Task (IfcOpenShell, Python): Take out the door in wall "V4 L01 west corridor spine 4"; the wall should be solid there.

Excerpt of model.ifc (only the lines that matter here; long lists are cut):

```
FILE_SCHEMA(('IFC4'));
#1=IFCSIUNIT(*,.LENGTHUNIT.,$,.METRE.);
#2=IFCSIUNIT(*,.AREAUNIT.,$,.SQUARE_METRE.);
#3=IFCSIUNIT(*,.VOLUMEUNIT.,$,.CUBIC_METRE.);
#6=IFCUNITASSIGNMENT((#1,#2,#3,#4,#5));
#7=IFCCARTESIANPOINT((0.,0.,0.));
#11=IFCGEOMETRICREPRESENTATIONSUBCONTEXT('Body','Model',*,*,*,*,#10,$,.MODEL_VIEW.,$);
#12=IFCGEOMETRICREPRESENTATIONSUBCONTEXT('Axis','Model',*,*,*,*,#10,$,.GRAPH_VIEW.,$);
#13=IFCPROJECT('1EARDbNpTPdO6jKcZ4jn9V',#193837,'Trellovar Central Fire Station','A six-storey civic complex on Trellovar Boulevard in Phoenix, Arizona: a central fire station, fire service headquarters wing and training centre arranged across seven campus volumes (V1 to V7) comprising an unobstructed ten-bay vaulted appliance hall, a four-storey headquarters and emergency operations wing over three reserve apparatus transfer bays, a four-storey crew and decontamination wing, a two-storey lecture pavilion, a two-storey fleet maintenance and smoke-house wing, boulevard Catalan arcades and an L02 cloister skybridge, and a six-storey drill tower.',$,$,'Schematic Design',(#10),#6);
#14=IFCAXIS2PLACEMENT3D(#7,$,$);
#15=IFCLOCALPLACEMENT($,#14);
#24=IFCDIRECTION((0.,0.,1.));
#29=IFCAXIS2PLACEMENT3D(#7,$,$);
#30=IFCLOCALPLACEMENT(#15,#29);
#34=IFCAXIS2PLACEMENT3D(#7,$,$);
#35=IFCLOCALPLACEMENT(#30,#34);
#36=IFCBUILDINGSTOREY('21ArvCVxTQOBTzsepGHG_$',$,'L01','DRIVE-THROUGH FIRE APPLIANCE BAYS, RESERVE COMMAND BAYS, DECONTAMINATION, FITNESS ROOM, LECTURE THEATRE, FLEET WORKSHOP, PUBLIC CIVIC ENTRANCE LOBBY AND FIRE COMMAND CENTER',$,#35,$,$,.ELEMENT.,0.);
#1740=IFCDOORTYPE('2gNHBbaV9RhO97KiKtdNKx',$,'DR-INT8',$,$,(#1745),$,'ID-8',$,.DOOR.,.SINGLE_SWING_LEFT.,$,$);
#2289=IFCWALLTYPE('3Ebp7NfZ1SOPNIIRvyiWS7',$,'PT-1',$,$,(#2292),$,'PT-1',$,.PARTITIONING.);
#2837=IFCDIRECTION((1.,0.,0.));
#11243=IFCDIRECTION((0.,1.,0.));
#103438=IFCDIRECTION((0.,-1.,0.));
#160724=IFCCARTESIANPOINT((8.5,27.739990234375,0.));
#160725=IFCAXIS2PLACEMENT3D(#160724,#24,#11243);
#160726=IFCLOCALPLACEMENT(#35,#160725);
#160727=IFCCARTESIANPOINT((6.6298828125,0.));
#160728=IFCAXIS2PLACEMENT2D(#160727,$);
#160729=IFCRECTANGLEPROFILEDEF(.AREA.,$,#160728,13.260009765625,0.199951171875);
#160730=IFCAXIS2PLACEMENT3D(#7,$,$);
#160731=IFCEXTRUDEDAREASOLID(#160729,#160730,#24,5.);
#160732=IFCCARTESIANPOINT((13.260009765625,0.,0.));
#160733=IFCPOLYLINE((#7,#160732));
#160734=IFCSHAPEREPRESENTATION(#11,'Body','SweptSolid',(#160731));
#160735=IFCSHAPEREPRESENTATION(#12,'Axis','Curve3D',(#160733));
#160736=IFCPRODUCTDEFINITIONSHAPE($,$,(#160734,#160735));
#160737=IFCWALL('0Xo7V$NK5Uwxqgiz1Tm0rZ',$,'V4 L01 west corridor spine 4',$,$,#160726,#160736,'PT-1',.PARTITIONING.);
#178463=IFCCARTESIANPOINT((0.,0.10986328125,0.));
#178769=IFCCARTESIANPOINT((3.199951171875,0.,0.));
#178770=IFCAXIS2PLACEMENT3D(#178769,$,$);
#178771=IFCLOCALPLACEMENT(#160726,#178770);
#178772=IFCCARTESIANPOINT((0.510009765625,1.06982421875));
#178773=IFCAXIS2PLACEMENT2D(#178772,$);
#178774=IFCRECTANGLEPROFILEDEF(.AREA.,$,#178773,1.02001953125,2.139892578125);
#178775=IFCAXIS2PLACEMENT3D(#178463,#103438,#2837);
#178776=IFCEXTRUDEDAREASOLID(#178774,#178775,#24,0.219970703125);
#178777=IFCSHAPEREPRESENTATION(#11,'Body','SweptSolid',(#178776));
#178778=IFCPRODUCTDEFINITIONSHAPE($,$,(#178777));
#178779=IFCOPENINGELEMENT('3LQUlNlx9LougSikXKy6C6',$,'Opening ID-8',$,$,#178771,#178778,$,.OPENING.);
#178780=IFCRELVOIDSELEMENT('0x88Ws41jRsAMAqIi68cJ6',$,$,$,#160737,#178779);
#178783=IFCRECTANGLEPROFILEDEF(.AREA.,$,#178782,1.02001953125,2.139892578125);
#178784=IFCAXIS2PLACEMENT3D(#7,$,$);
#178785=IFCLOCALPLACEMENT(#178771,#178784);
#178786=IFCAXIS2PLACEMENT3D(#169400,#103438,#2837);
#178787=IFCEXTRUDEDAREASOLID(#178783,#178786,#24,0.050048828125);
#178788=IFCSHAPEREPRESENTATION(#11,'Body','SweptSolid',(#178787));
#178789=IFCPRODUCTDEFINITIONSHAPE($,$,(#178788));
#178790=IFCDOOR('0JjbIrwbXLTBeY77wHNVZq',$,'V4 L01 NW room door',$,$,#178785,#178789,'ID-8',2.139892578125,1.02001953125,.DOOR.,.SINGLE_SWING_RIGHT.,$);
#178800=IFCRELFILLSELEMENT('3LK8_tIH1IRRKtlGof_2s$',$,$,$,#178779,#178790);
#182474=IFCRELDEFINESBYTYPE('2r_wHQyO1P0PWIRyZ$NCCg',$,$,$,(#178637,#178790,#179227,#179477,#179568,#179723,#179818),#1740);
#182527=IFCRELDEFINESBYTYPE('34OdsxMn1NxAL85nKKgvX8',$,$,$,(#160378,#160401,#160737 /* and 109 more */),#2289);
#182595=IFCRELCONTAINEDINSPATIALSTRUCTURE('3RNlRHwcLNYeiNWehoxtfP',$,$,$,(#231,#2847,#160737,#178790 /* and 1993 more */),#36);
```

```python
import ifcopenshell
import ifcopenshell.api.feature
import ifcopenshell.api.root
import ifcopenshell.geom
import ifcopenshell.util.shape

model = ifcopenshell.open("model.ifc")
settings = ifcopenshell.geom.settings()


def volume(element):
    """Net volume in cubic metres, openings subtracted."""
    shape = ifcopenshell.geom.create_shape(settings, element)
    return ifcopenshell.util.shape.get_volume(shape.geometry)


door = model.by_guid("0JjbIrwbXLTBeY77wHNVZq")
opening = door.FillsVoids[0].RelatingOpeningElement
wall = opening.VoidsElements[0].RelatingBuildingElement
before = volume(wall)

ifcopenshell.api.root.remove_product(model, product=door)
ifcopenshell.api.feature.remove_feature(model, feature=opening)

after = volume(wall)

print(f"wall volume {before:.3f} -> {after:.3f} m3")

model.write("model-out.ifc")
```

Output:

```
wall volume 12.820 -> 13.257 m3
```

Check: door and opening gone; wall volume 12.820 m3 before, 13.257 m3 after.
